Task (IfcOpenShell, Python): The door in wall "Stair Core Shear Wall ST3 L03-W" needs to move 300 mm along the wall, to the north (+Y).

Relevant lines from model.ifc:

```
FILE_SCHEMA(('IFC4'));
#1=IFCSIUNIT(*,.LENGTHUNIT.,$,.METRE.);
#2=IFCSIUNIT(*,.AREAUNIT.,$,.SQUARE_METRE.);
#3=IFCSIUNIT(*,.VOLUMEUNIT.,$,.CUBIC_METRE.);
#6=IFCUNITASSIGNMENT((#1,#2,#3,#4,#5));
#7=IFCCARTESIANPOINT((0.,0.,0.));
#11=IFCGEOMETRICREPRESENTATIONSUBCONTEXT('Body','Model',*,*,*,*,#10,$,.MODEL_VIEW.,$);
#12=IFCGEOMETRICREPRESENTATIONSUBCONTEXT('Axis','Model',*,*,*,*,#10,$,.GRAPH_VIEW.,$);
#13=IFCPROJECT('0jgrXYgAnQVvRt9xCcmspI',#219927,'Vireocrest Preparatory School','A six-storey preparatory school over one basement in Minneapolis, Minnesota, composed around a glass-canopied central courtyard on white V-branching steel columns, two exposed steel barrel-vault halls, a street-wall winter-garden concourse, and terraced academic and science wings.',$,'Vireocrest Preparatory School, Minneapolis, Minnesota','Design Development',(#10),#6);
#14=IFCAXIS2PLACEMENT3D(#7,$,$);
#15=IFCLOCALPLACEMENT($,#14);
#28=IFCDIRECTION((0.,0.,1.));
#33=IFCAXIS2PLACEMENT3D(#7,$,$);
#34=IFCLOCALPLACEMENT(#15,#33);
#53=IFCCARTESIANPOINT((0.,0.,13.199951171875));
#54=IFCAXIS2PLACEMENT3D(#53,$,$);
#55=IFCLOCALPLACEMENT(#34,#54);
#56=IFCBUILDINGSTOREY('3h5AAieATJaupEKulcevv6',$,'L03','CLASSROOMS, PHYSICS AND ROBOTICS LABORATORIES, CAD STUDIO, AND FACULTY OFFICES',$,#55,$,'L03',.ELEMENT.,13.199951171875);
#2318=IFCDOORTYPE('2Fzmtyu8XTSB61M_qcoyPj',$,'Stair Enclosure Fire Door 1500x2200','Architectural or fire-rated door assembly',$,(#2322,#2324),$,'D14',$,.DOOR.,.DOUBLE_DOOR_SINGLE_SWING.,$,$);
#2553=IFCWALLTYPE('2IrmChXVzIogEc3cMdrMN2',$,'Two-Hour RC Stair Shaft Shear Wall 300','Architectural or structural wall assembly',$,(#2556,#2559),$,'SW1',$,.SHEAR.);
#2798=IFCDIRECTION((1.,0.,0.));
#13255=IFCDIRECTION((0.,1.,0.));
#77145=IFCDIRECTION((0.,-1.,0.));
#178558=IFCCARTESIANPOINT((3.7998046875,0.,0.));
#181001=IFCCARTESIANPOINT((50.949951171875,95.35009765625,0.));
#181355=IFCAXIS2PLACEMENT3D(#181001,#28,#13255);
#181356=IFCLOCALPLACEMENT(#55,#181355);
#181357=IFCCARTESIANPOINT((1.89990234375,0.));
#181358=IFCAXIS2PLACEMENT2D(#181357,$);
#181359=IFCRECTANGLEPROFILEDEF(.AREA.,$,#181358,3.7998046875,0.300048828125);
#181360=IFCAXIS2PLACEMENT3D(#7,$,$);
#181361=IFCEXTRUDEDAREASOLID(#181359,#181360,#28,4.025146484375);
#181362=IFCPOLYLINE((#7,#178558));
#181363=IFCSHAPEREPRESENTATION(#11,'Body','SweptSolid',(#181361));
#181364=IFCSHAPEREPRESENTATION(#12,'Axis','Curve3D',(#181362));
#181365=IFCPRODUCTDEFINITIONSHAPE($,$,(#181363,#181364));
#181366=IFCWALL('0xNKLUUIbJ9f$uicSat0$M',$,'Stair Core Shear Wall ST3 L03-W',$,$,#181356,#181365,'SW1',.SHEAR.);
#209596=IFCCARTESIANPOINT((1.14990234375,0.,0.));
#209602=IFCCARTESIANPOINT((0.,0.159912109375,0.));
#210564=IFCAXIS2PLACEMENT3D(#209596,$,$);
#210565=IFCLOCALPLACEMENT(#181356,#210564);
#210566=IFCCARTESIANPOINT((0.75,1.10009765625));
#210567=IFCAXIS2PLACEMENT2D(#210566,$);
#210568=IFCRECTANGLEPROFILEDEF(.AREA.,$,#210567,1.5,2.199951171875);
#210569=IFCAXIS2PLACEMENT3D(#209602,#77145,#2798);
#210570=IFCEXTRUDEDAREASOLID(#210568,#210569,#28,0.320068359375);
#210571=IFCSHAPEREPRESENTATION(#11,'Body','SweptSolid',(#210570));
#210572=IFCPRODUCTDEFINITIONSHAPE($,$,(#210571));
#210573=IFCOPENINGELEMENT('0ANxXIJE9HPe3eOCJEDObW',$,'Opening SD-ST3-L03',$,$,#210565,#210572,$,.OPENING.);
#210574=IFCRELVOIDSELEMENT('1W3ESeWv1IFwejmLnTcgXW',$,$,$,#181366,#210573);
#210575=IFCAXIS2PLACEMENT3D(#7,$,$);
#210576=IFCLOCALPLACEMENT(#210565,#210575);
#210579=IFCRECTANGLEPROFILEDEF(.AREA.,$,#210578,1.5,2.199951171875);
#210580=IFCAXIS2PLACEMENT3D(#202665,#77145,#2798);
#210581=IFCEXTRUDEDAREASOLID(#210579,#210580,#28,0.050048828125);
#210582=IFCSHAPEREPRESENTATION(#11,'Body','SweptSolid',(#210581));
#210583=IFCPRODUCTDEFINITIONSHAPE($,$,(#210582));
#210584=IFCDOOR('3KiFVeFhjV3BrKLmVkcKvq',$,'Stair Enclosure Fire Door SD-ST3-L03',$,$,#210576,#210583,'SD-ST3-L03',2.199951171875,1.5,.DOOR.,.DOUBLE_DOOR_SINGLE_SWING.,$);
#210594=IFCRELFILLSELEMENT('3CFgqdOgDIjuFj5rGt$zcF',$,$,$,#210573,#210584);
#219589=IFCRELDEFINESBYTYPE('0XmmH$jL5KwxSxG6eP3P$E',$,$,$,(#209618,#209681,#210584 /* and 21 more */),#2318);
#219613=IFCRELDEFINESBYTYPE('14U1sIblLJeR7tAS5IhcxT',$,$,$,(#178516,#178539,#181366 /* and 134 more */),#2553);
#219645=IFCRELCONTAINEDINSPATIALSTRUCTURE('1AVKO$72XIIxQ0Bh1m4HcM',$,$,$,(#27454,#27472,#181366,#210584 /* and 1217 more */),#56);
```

```python
import ifcopenshell
import ifcopenshell.api.geometry
import ifcopenshell.util.placement
import ifcopenshell.util.unit

model = ifcopenshell.open("model.ifc")
unit_scale = ifcopenshell.util.unit.calculate_unit_scale(model)

door = model.by_guid("3KiFVeFhjV3BrKLmVkcKvq")
opening = door.FillsVoids[0].RelatingOpeningElement
wall = opening.VoidsElements[0].RelatingBuildingElement

wall_matrix = ifcopenshell.util.placement.get_local_placement(wall.ObjectPlacement)
shift = wall_matrix[:3, 0] * 0.3 / unit_scale
before = ifcopenshell.util.placement.get_local_placement(door.ObjectPlacement)[:3, 3].copy()

# The door is placed relative to its opening, so it follows when the opening moves.
matrix = ifcopenshell.util.placement.get_local_placement(opening.ObjectPlacement)
matrix[:3, 3] += shift
ifcopenshell.api.geometry.edit_object_placement(
    model, product=opening, matrix=matrix, is_si=False, should_transform_children=True
)

after = ifcopenshell.util.placement.get_local_placement(door.ObjectPlacement)[:3, 3]
print("door moved by", (after - before).round(3) + 0.0)

model.write("model_edited.ifc")
```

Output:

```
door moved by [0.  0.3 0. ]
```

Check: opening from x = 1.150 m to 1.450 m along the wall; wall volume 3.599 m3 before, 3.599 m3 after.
